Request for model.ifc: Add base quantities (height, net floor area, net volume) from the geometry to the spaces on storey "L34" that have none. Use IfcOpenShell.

First a look at what the model holds.

```python
import ifcopenshell
import ifcopenshell.util.element
import ifcopenshell.util.unit

model = ifcopenshell.open("model.ifc")
print(model.schema)
for unit_type in ("LENGTHUNIT", "AREAUNIT", "VOLUMEUNIT"):
    print(unit_type, ifcopenshell.util.unit.calculate_unit_scale(model, unit_type))
storey = next(s for s in model.by_type("IfcBuildingStorey") if s.Name == "L34")
spaces = [e for e in ifcopenshell.util.element.get_decomposition(storey) if e.is_a("IfcSpace")]
for e in sorted(spaces, key=lambda e: e.id()):
    print(e.id(), e.is_a(), e.Name, list(ifcopenshell.util.element.get_psets(e, qtos_only=True)), sep=" | ")
```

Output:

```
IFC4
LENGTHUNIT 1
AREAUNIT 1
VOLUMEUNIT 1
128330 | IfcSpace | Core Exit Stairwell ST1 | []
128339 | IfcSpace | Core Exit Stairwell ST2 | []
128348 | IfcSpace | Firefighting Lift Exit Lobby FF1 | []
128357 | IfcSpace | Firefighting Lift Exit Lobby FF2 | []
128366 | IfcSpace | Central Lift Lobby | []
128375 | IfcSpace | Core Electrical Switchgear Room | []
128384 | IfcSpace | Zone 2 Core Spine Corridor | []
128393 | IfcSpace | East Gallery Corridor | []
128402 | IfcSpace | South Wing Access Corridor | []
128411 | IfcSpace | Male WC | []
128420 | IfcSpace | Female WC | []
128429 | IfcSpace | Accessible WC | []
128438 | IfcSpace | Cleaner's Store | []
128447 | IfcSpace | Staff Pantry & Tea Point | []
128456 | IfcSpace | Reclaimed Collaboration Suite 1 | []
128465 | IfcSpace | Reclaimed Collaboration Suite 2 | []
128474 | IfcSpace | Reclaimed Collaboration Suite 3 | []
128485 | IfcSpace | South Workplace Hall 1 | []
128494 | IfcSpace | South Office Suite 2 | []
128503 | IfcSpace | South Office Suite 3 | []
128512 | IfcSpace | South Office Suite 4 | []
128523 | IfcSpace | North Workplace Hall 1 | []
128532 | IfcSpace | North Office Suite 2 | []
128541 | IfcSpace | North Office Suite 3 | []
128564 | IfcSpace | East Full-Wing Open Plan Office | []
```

```python
import ifcopenshell
import ifcopenshell.api.pset
import ifcopenshell.geom
import ifcopenshell.util.element
import ifcopenshell.util.shape
import ifcopenshell.util.unit

model = ifcopenshell.open("model.ifc")
unit_scale = ifcopenshell.util.unit.calculate_unit_scale(model)
area_scale = ifcopenshell.util.unit.calculate_unit_scale(model, "AREAUNIT")
volume_scale = ifcopenshell.util.unit.calculate_unit_scale(model, "VOLUMEUNIT")
settings = ifcopenshell.geom.settings()

storey = next(s for s in model.by_type("IfcBuildingStorey") if s.Name == "L34")
spaces = [e for e in ifcopenshell.util.element.get_decomposition(storey) if e.is_a("IfcSpace")]

for e in sorted(spaces, key=lambda e: e.id()):
    if ifcopenshell.util.element.get_psets(e, qtos_only=True, should_inherit=False):
        continue
    # Geometry comes back in metres, in the element's own axes.
    shape = ifcopenshell.geom.create_shape(settings, e)
    values = {
        "Height": ifcopenshell.util.shape.get_z(shape.geometry) / unit_scale,
        "NetFloorArea": ifcopenshell.util.shape.get_footprint_area(shape.geometry) / area_scale,
        "NetVolume": ifcopenshell.util.shape.get_volume(shape.geometry) / volume_scale,
    }
    qto = ifcopenshell.api.pset.add_qto(model, product=e, name="Qto_SpaceBaseQuantities")
    ifcopenshell.api.pset.edit_qto(model, qto=qto, properties=values)
    print(e.id(), {k: round(v, 3) for k, v in values.items()})

model.write("model_v2.ifc")
```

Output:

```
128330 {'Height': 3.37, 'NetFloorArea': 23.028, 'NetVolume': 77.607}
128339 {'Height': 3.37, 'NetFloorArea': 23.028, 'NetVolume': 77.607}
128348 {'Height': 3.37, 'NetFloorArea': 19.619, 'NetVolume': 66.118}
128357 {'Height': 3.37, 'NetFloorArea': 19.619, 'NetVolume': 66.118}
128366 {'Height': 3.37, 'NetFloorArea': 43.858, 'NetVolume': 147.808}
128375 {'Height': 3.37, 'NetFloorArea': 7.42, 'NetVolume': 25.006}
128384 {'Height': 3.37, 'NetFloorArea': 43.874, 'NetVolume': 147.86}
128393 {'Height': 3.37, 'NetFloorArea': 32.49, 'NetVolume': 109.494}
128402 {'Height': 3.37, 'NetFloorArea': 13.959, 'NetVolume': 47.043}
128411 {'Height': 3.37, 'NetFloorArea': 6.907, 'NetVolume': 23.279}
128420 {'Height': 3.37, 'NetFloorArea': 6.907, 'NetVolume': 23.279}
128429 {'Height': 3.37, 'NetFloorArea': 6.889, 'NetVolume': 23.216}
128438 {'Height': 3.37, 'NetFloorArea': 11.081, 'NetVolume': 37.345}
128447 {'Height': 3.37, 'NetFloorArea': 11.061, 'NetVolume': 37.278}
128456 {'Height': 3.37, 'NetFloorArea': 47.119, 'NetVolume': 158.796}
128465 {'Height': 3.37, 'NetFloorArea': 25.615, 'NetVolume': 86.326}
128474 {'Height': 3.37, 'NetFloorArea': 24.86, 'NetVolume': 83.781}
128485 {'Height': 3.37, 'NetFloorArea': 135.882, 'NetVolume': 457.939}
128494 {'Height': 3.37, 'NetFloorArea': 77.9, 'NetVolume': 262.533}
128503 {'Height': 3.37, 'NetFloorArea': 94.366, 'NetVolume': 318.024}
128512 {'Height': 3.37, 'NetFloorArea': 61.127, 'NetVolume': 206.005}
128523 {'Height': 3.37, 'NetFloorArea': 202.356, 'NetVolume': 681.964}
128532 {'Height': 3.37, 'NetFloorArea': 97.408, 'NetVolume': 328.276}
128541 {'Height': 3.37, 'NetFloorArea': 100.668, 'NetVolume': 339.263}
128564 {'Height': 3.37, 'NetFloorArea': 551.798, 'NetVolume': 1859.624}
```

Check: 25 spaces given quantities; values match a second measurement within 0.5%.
